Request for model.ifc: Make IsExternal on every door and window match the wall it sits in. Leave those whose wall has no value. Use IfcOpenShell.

First a look at what the model holds.

```python
import ifcopenshell
import ifcopenshell.util.element

model = ifcopenshell.open("model.ifc")
print(model.schema)
seen = {}
for e in model.by_type("IfcDoor") + model.by_type("IfcWindow"):
    if not e.FillsVoids:
        continue
    host = e.FillsVoids[0].RelatingOpeningElement.VoidsElements[0].RelatingBuildingElement
    own = ifcopenshell.util.element.get_pset(e, f"Pset_{e.is_a()[3:].removesuffix('StandardCase')}Common", "IsExternal")
    wall = ifcopenshell.util.element.get_pset(host, "Pset_WallCommon", "IsExternal")
    seen[e.is_a(), own, wall] = seen.get((e.is_a(), own, wall), 0) + 1
for (cls, own, wall), count in sorted(seen.items(), key=str):
    print(count, cls, "IsExternal:", own, "| host wall:", wall)
```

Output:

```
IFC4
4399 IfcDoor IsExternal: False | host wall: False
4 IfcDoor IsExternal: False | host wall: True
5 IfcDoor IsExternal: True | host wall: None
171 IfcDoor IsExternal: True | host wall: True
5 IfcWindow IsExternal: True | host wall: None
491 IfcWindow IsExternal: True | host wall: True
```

```python
import ifcopenshell
import ifcopenshell.api.pset
import ifcopenshell.util.element

model = ifcopenshell.open("model.ifc")

count = 0
for ifc_class, pset_name in (("IfcDoor", "Pset_DoorCommon"), ("IfcWindow", "Pset_WindowCommon")):
    for e in model.by_type(ifc_class):
        if not e.FillsVoids:
            continue
        host = e.FillsVoids[0].RelatingOpeningElement.VoidsElements[0].RelatingBuildingElement
        external = ifcopenshell.util.element.get_pset(host, "Pset_WallCommon", "IsExternal")
        if external is None or ifcopenshell.util.element.get_pset(e, pset_name, "IsExternal") == external:
            continue
        pset = ifcopenshell.api.pset.add_pset(model, product=e, name=pset_name)
        ifcopenshell.api.pset.edit_pset(model, pset=pset, properties={"IsExternal": external})
        count += 1

print(count, "updated")

model.write("model_updated.ifc")
```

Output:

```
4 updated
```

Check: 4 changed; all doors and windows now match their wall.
